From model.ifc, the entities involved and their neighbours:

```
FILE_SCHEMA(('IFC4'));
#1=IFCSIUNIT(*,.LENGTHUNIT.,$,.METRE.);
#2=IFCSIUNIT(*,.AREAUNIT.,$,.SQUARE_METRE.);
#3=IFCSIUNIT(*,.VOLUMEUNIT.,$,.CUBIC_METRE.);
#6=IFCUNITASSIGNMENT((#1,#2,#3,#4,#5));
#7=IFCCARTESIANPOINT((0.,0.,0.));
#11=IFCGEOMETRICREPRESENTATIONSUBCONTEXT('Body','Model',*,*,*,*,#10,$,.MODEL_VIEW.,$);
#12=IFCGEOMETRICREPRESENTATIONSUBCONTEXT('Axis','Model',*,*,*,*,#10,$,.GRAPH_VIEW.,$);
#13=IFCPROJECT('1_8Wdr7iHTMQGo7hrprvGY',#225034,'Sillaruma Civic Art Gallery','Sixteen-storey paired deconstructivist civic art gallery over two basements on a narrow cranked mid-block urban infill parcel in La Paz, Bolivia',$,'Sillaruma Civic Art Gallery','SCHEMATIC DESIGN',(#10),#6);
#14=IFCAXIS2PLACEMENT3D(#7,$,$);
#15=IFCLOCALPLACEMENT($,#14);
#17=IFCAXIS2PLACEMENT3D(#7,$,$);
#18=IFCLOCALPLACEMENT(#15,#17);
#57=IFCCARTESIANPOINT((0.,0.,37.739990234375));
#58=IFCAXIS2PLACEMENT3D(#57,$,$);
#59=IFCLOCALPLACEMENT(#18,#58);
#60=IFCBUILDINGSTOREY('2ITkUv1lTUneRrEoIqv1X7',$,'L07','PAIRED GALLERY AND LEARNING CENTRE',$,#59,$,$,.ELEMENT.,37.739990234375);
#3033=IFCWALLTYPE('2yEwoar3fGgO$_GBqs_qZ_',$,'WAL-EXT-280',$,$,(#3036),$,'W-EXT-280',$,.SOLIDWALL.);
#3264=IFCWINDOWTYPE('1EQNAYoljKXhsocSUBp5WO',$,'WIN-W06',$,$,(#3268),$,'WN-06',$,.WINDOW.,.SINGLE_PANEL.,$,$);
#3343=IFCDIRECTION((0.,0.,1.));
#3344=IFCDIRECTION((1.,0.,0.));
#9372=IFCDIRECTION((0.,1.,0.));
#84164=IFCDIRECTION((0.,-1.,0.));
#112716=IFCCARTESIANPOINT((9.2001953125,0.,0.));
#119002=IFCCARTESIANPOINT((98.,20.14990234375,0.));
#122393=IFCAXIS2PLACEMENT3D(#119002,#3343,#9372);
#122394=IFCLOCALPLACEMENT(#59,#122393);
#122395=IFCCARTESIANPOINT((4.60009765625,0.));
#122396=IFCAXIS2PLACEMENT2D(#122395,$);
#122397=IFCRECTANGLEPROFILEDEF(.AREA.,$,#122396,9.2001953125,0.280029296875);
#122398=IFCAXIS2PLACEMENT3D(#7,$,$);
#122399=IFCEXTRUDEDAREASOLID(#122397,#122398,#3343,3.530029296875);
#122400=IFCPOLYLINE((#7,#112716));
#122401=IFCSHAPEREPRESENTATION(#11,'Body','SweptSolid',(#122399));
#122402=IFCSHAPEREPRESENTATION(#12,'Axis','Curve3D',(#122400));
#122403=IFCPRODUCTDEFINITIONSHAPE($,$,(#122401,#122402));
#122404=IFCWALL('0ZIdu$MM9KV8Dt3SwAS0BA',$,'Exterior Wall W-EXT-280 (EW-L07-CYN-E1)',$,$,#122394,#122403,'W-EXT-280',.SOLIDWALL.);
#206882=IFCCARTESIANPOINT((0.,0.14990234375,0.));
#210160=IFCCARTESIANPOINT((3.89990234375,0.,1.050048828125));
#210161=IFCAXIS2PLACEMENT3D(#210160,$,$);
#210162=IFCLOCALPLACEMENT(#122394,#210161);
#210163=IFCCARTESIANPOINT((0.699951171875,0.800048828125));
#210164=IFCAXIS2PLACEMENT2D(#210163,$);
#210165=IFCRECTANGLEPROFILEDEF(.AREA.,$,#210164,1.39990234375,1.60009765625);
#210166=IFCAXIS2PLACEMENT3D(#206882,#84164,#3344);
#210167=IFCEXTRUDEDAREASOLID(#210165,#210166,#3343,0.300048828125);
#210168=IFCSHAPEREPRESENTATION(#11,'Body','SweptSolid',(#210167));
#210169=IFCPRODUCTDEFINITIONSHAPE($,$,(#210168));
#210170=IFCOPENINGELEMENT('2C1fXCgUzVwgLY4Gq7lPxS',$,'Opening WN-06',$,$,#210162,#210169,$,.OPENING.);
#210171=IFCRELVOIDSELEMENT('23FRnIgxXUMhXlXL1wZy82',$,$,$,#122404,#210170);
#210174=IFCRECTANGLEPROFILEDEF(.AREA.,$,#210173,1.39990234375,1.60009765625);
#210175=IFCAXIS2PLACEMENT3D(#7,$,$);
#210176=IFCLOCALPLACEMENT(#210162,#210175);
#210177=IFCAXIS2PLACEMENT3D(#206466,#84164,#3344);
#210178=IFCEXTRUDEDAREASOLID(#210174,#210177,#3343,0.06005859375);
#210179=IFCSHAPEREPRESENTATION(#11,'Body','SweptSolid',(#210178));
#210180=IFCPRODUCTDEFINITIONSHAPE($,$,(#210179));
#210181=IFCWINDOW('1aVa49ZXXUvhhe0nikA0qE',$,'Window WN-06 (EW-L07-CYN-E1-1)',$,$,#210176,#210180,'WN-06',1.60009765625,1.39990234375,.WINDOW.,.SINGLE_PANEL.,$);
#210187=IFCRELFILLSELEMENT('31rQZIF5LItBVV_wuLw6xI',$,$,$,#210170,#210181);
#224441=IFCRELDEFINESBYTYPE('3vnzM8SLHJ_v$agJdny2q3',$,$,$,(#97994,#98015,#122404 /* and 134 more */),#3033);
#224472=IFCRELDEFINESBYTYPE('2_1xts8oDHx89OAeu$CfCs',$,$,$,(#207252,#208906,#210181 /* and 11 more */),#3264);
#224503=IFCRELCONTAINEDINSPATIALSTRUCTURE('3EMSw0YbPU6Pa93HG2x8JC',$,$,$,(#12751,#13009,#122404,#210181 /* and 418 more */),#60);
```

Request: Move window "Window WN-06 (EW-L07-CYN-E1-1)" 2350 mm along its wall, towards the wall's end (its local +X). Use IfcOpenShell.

```python
import ifcopenshell
import ifcopenshell.api.geometry
import ifcopenshell.util.placement
import ifcopenshell.util.unit

model = ifcopenshell.open("model.ifc")
unit_scale = ifcopenshell.util.unit.calculate_unit_scale(model)

window = model.by_id(210181)
opening = window.FillsVoids[0].RelatingOpeningElement
wall = opening.VoidsElements[0].RelatingBuildingElement

wall_matrix = ifcopenshell.util.placement.get_local_placement(wall.ObjectPlacement)
shift = wall_matrix[:3, 0] * 2.35 / unit_scale
before = ifcopenshell.util.placement.get_local_placement(window.ObjectPlacement)[:3, 3].copy()

# The window is placed relative to its opening, so it follows when the opening moves.
matrix = ifcopenshell.util.placement.get_local_placement(opening.ObjectPlacement)
matrix[:3, 3] += shift
ifcopenshell.api.geometry.edit_object_placement(
    model, product=opening, matrix=matrix, is_si=False, should_transform_children=True
)

after = ifcopenshell.util.placement.get_local_placement(window.ObjectPlacement)[:3, 3]
print("window moved by", (after - before).round(3) + 0.0)

model.write("model_updated.ifc")
```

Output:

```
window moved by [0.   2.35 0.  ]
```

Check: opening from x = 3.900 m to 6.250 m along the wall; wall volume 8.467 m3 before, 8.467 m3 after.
